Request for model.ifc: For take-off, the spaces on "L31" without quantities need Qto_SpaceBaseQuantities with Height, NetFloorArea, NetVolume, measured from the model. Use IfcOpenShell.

First a look at what the model holds.

```python
import ifcopenshell
import ifcopenshell.util.element
import ifcopenshell.util.unit

model = ifcopenshell.open("model.ifc")
print(model.schema)
for unit_type in ("LENGTHUNIT", "AREAUNIT", "VOLUMEUNIT"):
    print(unit_type, ifcopenshell.util.unit.calculate_unit_scale(model, unit_type))
storey = next(s for s in model.by_type("IfcBuildingStorey") if s.Name == "L31")
spaces = [e for e in ifcopenshell.util.element.get_decomposition(storey) if e.is_a("IfcSpace")]
for e in sorted(spaces, key=lambda e: e.id()):
    print(e.id(), e.is_a(), e.Name, list(ifcopenshell.util.element.get_psets(e, qtos_only=True)), sep=" | ")
```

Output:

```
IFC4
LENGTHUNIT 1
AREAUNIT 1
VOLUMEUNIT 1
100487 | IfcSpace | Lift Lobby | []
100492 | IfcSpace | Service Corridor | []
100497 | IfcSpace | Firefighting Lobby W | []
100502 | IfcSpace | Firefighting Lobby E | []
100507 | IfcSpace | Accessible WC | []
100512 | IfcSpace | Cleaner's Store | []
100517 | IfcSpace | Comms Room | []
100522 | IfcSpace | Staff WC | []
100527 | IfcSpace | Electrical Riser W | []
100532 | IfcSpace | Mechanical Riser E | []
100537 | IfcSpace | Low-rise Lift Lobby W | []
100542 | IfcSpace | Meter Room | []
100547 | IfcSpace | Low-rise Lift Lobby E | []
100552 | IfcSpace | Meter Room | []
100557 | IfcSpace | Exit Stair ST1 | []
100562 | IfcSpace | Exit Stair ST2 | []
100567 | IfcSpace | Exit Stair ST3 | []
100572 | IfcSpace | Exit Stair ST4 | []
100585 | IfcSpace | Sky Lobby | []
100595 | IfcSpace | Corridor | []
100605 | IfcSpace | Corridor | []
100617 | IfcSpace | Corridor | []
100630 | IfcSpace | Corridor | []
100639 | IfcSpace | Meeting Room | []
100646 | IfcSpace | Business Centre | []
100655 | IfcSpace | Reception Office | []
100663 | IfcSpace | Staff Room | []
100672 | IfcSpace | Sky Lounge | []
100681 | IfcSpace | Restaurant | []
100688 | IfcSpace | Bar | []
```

```python
import ifcopenshell
import ifcopenshell.api.pset
import ifcopenshell.geom
import ifcopenshell.util.element
import ifcopenshell.util.shape
import ifcopenshell.util.unit

model = ifcopenshell.open("model.ifc")
unit_scale = ifcopenshell.util.unit.calculate_unit_scale(model)
area_scale = ifcopenshell.util.unit.calculate_unit_scale(model, "AREAUNIT")
volume_scale = ifcopenshell.util.unit.calculate_unit_scale(model, "VOLUMEUNIT")
settings = ifcopenshell.geom.settings()

storey = next(s for s in model.by_type("IfcBuildingStorey") if s.Name == "L31")
spaces = [e for e in ifcopenshell.util.element.get_decomposition(storey) if e.is_a("IfcSpace")]

for e in sorted(spaces, key=lambda e: e.id()):
    if ifcopenshell.util.element.get_psets(e, qtos_only=True, should_inherit=False):
        continue
    # Geometry comes back in metres, in the element's own axes.
    shape = ifcopenshell.geom.create_shape(settings, e)
    values = {
        "Height": ifcopenshell.util.shape.get_z(shape.geometry) / unit_scale,
        "NetFloorArea": ifcopenshell.util.shape.get_footprint_area(shape.geometry) / area_scale,
        "NetVolume": ifcopenshell.util.shape.get_volume(shape.geometry) / volume_scale,
    }
    qto = ifcopenshell.api.pset.add_qto(model, product=e, name="Qto_SpaceBaseQuantities")
    ifcopenshell.api.pset.edit_qto(model, qto=qto, properties=values)
    print(e.id(), {k: round(v, 3) for k, v in values.items()})

model.write("model_edited.ifc")
```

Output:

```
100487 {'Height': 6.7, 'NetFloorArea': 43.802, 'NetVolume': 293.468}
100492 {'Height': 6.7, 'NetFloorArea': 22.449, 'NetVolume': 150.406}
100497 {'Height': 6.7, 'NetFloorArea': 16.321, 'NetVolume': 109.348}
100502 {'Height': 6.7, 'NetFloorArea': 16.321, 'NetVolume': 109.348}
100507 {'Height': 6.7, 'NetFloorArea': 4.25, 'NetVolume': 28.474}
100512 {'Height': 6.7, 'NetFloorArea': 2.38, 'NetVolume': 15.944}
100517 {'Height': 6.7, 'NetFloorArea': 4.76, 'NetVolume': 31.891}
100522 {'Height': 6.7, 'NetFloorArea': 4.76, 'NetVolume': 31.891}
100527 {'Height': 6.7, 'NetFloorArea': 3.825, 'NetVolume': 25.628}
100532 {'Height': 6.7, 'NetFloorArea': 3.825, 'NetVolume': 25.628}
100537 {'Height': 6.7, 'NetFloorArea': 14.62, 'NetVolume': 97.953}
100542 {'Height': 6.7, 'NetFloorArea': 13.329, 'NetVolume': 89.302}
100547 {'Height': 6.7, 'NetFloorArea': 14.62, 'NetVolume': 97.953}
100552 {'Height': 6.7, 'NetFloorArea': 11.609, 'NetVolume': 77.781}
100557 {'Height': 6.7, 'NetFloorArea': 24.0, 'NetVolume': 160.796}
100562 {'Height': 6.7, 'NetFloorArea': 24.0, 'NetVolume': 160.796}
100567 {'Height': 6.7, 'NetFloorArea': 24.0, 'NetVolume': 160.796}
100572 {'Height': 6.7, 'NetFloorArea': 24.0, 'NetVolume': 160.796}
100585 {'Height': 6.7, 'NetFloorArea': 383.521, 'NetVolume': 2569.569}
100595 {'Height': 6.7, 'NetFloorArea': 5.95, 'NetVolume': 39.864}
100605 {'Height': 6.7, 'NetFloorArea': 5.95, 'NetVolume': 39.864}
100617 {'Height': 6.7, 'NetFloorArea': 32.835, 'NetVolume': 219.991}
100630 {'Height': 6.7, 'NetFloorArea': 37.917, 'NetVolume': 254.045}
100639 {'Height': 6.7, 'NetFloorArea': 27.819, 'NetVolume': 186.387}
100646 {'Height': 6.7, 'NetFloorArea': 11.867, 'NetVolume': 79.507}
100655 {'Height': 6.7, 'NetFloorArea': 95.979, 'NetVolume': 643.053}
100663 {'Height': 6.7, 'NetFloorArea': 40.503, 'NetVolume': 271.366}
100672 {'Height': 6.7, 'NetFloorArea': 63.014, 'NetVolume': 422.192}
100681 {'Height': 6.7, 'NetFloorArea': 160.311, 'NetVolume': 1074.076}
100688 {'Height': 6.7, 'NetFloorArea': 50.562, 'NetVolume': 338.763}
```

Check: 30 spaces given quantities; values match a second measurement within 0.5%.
